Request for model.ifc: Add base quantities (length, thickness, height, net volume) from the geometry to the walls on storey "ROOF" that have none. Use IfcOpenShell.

First a look at what the model holds.

```python
import ifcopenshell
import ifcopenshell.util.element
import ifcopenshell.util.unit

model = ifcopenshell.open("model.ifc")
print(model.schema)
for unit_type in ("LENGTHUNIT", "AREAUNIT", "VOLUMEUNIT"):
    print(unit_type, ifcopenshell.util.unit.calculate_unit_scale(model, unit_type))
storey = next(s for s in model.by_type("IfcBuildingStorey") if s.Name == "ROOF")
walls = [e for e in ifcopenshell.util.element.get_decomposition(storey) if e.is_a("IfcWall")]
for e in sorted(walls, key=lambda e: e.id()):
    print(e.id(), e.is_a(), e.Name, list(ifcopenshell.util.element.get_psets(e, qtos_only=True)), sep=" | ")
```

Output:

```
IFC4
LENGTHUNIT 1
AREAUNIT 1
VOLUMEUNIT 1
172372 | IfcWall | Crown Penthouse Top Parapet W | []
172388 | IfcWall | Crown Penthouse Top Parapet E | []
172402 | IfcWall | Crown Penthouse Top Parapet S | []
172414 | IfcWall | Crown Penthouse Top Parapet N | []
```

```python
import ifcopenshell
import ifcopenshell.api.pset
import ifcopenshell.geom
import ifcopenshell.util.element
import ifcopenshell.util.shape
import ifcopenshell.util.unit

model = ifcopenshell.open("model.ifc")
unit_scale = ifcopenshell.util.unit.calculate_unit_scale(model)
volume_scale = ifcopenshell.util.unit.calculate_unit_scale(model, "VOLUMEUNIT")
settings = ifcopenshell.geom.settings()

storey = next(s for s in model.by_type("IfcBuildingStorey") if s.Name == "ROOF")
walls = [e for e in ifcopenshell.util.element.get_decomposition(storey) if e.is_a("IfcWall")]

for e in sorted(walls, key=lambda e: e.id()):
    if ifcopenshell.util.element.get_psets(e, qtos_only=True, should_inherit=False):
        continue
    # Geometry comes back in metres, in the element's own axes.
    shape = ifcopenshell.geom.create_shape(settings, e)
    values = {
        "Length": ifcopenshell.util.shape.get_x(shape.geometry) / unit_scale,
        "Width": ifcopenshell.util.shape.get_y(shape.geometry) / unit_scale,
        "Height": ifcopenshell.util.shape.get_z(shape.geometry) / unit_scale,
        "NetVolume": ifcopenshell.util.shape.get_volume(shape.geometry) / volume_scale,
    }
    qto = ifcopenshell.api.pset.add_qto(model, product=e, name="Qto_WallBaseQuantities")
    ifcopenshell.api.pset.edit_qto(model, qto=qto, properties=values)
    print(e.id(), {k: round(v, 3) for k, v in values.items()})

model.write("model_rev.ifc")
```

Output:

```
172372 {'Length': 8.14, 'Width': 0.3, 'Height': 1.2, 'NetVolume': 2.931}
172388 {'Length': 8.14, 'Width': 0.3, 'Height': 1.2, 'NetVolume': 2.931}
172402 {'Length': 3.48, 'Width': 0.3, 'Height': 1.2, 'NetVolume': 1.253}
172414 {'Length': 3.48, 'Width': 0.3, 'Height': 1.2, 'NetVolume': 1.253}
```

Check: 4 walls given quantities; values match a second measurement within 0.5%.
